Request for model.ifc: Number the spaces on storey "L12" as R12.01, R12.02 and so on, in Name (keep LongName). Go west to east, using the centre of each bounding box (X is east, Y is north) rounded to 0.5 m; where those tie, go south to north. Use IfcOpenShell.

First a look at what the model holds.

```python
import ifcopenshell
import ifcopenshell.util.element
import ifcopenshell.util.placement

model = ifcopenshell.open("model.ifc")
print(model.schema)
storey = next(s for s in model.by_type("IfcBuildingStorey") if s.Name == "L12")
spaces = [e for e in ifcopenshell.util.element.get_decomposition(storey) if e.is_a("IfcSpace")]
for e in sorted(spaces, key=lambda e: e.id()):
    origin = ifcopenshell.util.placement.get_local_placement(e.ObjectPlacement)[:3, 3]
    print(e.id(), e.Name, e.LongName, origin.round(2) + 0.0, sep=" | ")
```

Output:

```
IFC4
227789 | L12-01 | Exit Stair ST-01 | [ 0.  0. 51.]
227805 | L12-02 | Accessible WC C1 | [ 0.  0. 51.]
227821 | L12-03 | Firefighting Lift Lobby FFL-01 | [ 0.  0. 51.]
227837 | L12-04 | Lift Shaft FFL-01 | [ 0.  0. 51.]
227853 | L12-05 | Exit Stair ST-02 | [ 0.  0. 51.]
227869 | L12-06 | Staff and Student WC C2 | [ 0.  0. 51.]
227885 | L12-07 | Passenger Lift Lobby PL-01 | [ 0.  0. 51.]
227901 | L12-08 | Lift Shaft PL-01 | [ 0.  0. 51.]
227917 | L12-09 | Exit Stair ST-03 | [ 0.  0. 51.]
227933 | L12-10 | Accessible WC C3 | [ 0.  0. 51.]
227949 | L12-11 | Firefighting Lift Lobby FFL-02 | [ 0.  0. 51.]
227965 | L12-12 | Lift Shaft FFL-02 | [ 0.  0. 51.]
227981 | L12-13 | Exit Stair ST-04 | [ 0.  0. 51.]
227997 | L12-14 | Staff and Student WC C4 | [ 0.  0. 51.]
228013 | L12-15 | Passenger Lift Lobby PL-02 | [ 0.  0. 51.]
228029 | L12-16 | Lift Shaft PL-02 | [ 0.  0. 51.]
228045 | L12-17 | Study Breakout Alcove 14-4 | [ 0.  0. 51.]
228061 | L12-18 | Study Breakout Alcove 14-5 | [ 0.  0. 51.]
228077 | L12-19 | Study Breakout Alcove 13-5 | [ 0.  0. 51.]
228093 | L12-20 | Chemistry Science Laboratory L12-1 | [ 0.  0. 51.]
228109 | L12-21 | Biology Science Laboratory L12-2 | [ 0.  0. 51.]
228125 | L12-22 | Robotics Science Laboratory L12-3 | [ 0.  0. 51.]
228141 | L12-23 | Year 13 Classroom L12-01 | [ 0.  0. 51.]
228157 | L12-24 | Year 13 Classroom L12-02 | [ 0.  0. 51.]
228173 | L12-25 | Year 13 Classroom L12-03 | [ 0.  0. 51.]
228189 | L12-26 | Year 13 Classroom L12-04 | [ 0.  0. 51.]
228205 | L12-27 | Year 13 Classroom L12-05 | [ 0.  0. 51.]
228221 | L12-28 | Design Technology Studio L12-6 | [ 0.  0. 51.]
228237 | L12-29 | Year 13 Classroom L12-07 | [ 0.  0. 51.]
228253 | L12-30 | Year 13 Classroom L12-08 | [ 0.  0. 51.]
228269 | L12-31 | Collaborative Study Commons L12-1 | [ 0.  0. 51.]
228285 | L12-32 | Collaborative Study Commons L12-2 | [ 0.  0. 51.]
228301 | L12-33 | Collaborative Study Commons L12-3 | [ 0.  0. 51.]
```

```python
import ifcopenshell
import ifcopenshell.geom
import ifcopenshell.util.element
import ifcopenshell.util.shape

model = ifcopenshell.open("model.ifc")
settings = ifcopenshell.geom.settings()
settings.set("use-world-coords", True)


def centre(element):
    shape = ifcopenshell.geom.create_shape(settings, element)
    return ifcopenshell.util.shape.get_bbox_centroid(shape.geometry)


storey = next(s for s in model.by_type("IfcBuildingStorey") if s.Name == "L12")
spaces = [e for e in ifcopenshell.util.element.get_decomposition(storey) if e.is_a("IfcSpace")]

# Insertion points can sit at a corner or the storey origin, so sort by the geometry (in metres).
centres = {e: centre(e) for e in spaces}
spaces.sort(key=lambda e: (round(centres[e][0] / 0.5), centres[e][1]))

for i, e in enumerate(spaces, start=1):
    number = f"R12.{i:02d}"
    e.Name = number
    print(e.id(), number)

model.write("model_edited.ifc")
```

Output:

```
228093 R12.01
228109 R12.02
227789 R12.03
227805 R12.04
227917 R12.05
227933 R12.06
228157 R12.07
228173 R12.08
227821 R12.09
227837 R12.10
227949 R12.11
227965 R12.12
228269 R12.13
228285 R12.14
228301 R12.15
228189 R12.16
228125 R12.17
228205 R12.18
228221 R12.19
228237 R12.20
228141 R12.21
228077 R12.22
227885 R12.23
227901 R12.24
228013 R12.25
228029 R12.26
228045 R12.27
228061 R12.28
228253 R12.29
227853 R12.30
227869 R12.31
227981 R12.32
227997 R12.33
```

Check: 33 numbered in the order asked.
